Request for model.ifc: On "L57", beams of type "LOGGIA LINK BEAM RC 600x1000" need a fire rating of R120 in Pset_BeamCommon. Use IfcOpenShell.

First a look at what the model holds.

```python
import ifcopenshell
import ifcopenshell.util.element

model = ifcopenshell.open("model.ifc")
print(model.schema)
storey = next(s for s in model.by_type("IfcBuildingStorey") if s.Name == "L57")
beams = [e for e in ifcopenshell.util.element.get_decomposition(storey) if e.is_a("IfcBeam")]
seen = {}
for e in beams:
    element_type = ifcopenshell.util.element.get_type(e)
    key = (element_type.Name if element_type != e and element_type else None, ifcopenshell.util.element.get_pset(e, "Pset_BeamCommon", "FireRating"))
    seen[key] = seen.get(key, 0) + 1
for (name, value), count in sorted(seen.items(), key=str):
    print(count, "x", name, "|", value)
```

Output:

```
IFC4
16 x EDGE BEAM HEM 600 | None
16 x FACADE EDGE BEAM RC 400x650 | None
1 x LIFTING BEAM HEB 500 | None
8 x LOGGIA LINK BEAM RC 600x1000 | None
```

```python
import ifcopenshell
import ifcopenshell.api.pset
import ifcopenshell.util.element

model = ifcopenshell.open("model.ifc")

storey = next(s for s in model.by_type("IfcBuildingStorey") if s.Name == "L57")
beams = [e for e in ifcopenshell.util.element.get_decomposition(storey) if e.is_a("IfcBeam")]

count = 0
for e in beams:
    element_type = ifcopenshell.util.element.get_type(e)
    if element_type in (None, e) or element_type.Name != "LOGGIA LINK BEAM RC 600x1000":
        continue
    # add_pset returns the element's existing set when there is one.
    pset = ifcopenshell.api.pset.add_pset(model, product=e, name="Pset_BeamCommon")
    ifcopenshell.api.pset.edit_pset(model, pset=pset, properties={"FireRating": "R120"})
    count += 1

print(count, "beams updated")

model.write("model_rev.ifc")
```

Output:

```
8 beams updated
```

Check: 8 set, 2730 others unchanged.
